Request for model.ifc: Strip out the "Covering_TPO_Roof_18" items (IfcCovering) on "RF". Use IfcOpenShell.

First a look at what the model holds.

```python
import ifcopenshell
import ifcopenshell.util.element

model = ifcopenshell.open("model.ifc")
print(model.schema)
storey = next(s for s in model.by_type("IfcBuildingStorey") if s.Name == "RF")
coverings = [e for e in ifcopenshell.util.element.get_decomposition(storey) if e.is_a("IfcCovering")]
seen = {}
for e in coverings:
    element_type = ifcopenshell.util.element.get_type(e)
    name = element_type.Name if element_type not in (None, e) else None
    seen[name] = seen.get(name, 0) + 1
for name, count in sorted(seen.items(), key=str):
    print(count, "x", name)
```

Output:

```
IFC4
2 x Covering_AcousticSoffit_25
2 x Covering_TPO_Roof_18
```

```python
import ifcopenshell
import ifcopenshell.api.root
import ifcopenshell.util.element

model = ifcopenshell.open("model.ifc")

storey = next(s for s in model.by_type("IfcBuildingStorey") if s.Name == "RF")
coverings = [e for e in ifcopenshell.util.element.get_decomposition(storey) if e.is_a("IfcCovering")]
targets = [e for e in coverings if (t := ifcopenshell.util.element.get_type(e)) not in (None, e) and t.Name == "Covering_TPO_Roof_18"]

for e in targets:
    ifcopenshell.api.root.remove_product(model, product=e)
print(len(targets), "removed")

model.write("model_v2.ifc")
```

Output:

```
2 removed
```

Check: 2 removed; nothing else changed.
